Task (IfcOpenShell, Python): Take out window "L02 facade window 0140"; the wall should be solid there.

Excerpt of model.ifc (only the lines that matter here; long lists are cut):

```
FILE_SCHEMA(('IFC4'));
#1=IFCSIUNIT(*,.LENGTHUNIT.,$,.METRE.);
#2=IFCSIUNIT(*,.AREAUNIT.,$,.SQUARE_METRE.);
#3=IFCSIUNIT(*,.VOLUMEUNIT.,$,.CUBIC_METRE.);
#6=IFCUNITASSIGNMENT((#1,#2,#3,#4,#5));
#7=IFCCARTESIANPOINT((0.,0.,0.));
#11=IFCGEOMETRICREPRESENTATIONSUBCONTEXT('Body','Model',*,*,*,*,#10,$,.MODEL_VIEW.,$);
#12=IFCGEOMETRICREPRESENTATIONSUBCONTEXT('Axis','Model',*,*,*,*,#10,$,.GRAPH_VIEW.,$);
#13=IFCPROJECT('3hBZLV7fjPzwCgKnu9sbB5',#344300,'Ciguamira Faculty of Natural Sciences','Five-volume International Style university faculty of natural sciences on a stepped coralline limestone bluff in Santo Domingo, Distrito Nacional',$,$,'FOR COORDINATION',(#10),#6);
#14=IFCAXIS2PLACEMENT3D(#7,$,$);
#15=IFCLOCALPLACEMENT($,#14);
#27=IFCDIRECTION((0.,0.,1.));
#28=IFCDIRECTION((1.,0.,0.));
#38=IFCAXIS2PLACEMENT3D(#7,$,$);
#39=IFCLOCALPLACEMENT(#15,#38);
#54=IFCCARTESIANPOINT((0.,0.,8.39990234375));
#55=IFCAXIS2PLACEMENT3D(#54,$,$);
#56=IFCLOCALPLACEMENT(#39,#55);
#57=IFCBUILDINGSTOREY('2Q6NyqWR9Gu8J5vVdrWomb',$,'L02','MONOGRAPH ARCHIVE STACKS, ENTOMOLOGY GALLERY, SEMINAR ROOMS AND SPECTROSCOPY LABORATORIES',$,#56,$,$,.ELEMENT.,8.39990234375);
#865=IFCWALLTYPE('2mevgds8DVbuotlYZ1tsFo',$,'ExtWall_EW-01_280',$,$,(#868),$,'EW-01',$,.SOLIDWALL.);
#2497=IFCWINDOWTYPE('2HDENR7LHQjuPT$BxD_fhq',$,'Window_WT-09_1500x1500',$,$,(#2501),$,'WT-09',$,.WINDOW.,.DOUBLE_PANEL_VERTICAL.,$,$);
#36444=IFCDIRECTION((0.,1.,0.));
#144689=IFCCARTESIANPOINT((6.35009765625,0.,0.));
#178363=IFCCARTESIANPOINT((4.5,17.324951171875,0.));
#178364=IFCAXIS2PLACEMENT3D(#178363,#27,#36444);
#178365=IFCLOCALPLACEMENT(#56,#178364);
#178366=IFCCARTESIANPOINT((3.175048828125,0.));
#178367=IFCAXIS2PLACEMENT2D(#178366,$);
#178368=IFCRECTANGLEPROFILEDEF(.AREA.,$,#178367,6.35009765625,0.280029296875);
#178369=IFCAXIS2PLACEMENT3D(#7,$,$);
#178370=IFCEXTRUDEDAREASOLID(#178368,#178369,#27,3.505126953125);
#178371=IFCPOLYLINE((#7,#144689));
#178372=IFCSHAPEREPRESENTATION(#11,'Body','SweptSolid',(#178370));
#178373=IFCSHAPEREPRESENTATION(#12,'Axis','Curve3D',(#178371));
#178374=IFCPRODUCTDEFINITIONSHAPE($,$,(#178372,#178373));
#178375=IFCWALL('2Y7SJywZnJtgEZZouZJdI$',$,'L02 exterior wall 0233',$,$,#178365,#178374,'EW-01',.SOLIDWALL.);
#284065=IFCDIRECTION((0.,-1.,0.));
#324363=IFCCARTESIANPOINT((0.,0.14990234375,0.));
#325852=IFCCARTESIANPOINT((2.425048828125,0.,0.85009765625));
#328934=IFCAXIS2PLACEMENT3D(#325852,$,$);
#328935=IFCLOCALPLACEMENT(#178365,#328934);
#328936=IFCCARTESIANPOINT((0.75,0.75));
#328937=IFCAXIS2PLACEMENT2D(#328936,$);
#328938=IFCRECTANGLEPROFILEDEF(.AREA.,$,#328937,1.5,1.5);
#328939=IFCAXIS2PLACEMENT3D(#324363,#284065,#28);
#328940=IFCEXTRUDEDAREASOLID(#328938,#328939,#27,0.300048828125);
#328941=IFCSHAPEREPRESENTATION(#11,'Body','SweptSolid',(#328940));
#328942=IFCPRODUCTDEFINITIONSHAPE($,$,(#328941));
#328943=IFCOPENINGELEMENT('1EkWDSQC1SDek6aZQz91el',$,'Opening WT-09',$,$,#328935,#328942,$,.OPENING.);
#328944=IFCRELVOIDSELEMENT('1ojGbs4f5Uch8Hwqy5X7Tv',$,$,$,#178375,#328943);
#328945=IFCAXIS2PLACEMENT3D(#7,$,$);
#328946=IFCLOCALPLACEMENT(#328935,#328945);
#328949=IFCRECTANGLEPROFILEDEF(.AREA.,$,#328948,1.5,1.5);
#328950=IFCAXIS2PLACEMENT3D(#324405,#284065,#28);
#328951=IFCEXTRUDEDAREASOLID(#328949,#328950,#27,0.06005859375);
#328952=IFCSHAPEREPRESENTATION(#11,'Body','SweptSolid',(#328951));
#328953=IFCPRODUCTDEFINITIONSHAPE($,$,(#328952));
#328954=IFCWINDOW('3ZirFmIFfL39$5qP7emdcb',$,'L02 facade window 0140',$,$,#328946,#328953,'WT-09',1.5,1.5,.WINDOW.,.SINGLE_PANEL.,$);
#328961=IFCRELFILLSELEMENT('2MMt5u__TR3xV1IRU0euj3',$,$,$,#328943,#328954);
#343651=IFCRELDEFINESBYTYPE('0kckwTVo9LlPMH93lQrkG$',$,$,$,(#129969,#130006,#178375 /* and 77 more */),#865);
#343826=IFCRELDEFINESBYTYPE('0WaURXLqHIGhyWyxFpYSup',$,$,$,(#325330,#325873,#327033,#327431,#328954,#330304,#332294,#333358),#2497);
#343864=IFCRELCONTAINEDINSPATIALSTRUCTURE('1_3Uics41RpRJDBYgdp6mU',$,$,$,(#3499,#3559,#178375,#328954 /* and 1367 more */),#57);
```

```python
import ifcopenshell
import ifcopenshell.api.feature
import ifcopenshell.api.root
import ifcopenshell.geom
import ifcopenshell.util.shape

model = ifcopenshell.open("model.ifc")
settings = ifcopenshell.geom.settings()


def volume(element):
    """Net volume in cubic metres, openings subtracted."""
    shape = ifcopenshell.geom.create_shape(settings, element)
    return ifcopenshell.util.shape.get_volume(shape.geometry)


window = model.by_guid("3ZirFmIFfL39$5qP7emdcb")
opening = window.FillsVoids[0].RelatingOpeningElement
wall = opening.VoidsElements[0].RelatingBuildingElement
before = volume(wall)

ifcopenshell.api.root.remove_product(model, product=window)
ifcopenshell.api.feature.remove_feature(model, feature=opening)

after = volume(wall)

print(f"wall volume {before:.3f} -> {after:.3f} m3")

model.write("model_edited.ifc")
```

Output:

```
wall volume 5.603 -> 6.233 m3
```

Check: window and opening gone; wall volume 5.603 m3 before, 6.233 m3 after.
